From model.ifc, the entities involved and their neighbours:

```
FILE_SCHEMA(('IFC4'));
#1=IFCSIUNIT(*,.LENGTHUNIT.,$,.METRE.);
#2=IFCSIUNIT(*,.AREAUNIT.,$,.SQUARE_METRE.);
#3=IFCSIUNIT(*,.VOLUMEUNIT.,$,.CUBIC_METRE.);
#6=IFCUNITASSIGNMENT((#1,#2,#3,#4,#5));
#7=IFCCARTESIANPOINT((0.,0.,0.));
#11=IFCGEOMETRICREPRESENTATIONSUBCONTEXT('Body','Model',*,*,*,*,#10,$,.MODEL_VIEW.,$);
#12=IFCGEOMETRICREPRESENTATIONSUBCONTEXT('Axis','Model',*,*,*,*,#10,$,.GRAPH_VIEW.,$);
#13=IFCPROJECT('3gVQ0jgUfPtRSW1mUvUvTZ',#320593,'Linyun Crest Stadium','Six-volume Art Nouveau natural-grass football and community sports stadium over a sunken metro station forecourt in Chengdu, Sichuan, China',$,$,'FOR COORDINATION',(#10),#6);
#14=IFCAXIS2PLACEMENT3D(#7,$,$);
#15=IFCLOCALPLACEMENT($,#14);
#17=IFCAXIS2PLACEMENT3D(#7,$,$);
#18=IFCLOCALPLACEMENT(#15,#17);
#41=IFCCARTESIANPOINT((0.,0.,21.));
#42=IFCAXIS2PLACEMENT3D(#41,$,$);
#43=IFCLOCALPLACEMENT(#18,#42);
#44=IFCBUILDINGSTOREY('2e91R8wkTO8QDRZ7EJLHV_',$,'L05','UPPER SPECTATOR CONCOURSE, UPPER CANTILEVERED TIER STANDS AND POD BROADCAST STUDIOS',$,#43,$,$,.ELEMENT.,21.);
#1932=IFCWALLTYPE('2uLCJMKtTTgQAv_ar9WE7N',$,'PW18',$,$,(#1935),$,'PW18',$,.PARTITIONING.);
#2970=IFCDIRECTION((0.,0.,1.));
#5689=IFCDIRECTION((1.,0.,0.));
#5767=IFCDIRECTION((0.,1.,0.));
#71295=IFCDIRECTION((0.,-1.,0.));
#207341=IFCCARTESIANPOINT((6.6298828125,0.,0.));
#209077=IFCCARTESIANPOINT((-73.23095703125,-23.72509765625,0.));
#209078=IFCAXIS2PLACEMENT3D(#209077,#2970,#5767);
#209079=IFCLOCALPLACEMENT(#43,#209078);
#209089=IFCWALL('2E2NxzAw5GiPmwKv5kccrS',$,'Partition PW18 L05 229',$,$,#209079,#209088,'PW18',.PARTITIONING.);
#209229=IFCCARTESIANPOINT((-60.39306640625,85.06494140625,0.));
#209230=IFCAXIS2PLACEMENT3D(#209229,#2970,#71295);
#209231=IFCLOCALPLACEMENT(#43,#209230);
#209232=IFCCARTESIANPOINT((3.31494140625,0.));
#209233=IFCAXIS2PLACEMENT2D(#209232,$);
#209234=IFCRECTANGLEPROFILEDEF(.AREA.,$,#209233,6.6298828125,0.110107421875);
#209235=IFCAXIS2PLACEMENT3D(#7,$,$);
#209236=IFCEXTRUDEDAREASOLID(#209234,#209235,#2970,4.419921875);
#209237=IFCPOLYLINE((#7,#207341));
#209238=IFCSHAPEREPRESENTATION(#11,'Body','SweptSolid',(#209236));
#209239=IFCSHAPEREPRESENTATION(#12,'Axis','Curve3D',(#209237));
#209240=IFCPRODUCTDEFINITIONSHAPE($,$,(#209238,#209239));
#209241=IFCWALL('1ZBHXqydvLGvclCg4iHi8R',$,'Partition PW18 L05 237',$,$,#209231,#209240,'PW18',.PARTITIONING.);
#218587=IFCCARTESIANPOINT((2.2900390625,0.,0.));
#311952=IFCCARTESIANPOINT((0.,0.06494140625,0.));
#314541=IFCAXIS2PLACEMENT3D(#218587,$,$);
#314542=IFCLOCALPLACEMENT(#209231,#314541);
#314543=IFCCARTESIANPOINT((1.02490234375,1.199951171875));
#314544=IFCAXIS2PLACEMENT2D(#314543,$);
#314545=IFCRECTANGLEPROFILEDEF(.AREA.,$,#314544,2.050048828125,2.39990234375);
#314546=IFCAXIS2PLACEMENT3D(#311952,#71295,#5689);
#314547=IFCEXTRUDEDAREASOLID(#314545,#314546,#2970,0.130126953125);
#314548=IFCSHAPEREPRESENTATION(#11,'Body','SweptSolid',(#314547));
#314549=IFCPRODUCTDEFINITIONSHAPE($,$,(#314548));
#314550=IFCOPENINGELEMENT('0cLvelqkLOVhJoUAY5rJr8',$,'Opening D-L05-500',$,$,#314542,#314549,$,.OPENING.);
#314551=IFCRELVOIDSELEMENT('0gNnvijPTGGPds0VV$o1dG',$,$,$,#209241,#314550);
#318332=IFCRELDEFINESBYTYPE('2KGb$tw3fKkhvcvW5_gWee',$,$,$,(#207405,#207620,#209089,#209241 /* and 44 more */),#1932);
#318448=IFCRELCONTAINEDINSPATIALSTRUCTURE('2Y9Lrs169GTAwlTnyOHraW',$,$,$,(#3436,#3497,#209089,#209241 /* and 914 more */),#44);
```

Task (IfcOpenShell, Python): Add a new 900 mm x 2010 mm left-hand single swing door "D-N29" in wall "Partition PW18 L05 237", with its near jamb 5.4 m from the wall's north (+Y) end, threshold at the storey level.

```python
import numpy as np
import ifcopenshell
import ifcopenshell.api.feature
import ifcopenshell.api.geometry
import ifcopenshell.api.root
import ifcopenshell.api.spatial
import ifcopenshell.geom
import ifcopenshell.util.element
import ifcopenshell.util.placement
import ifcopenshell.util.representation
import ifcopenshell.util.shape
import ifcopenshell.util.unit

model = ifcopenshell.open("model.ifc")
unit_scale = ifcopenshell.util.unit.calculate_unit_scale(model)
settings = ifcopenshell.geom.settings()


def volume(element):
    """Net volume in cubic metres, openings subtracted."""
    shape = ifcopenshell.geom.create_shape(settings, element)
    return ifcopenshell.util.shape.get_volume(shape.geometry)


wall = model.by_id(209241)
storey = ifcopenshell.util.element.get_container(wall, ifc_class="IfcBuildingStorey")
context = ifcopenshell.util.representation.get_context(model, "Model", "Body", "MODEL_VIEW")
before = volume(wall)

width, height, from_end, sill = 0.9, 2.01, 5.4, 0.0  # metres

# The wall runs along its own X axis, and the end named is its -X end.
wall_shape = ifcopenshell.geom.create_shape(settings, wall)
x, y, z = ifcopenshell.util.shape.get_vertices(wall_shape.geometry).T
start = x.min() + from_end
face, thickness = float(y.min()), float(y.max() - y.min())
wall_matrix = ifcopenshell.util.placement.get_local_placement(wall.ObjectPlacement)
level = ifcopenshell.util.placement.get_local_placement(storey.ObjectPlacement)[2, 3]


def in_wall(x, y):
    """Placement at x, y metres in the wall's axes, at sill height."""
    matrix = wall_matrix.copy()
    matrix[:, 3] = wall_matrix @ np.array([x / unit_scale, y / unit_scale, 0.0, 1.0])
    matrix[2, 3] = level + sill / unit_scale
    return matrix


# Opening: a box that overshoots both wall faces by 50 mm.
opening = ifcopenshell.api.root.create_entity(model, ifc_class="IfcOpeningElement", predefined_type="OPENING")
box = ifcopenshell.api.geometry.add_wall_representation(
    model, context=context, length=width, height=height, thickness=thickness + 0.1
)
ifcopenshell.api.geometry.assign_representation(model, product=opening, representation=box)
ifcopenshell.api.geometry.edit_object_placement(model, product=opening, matrix=in_wall(start, face - 0.05), is_si=False)
ifcopenshell.api.feature.add_feature(model, feature=opening, element=wall)

door = ifcopenshell.api.root.create_entity(model, ifc_class="IfcDoor", name="D-N29", predefined_type="DOOR")
door.OverallWidth, door.OverallHeight = width / unit_scale, height / unit_scale
door.OperationType = "SINGLE_SWING_LEFT"
body = ifcopenshell.api.geometry.add_door_representation(
    model,
    context=context,
    overall_width=door.OverallWidth,
    overall_height=door.OverallHeight,
    operation_type="SINGLE_SWING_LEFT",
    lining_properties={"LiningDepth": thickness / unit_scale, "ThresholdDepth": thickness / unit_scale},
)
ifcopenshell.api.geometry.assign_representation(model, product=door, representation=body)
ifcopenshell.api.spatial.assign_container(model, products=[door], relating_structure=storey)
ifcopenshell.api.feature.add_filling(model, opening=opening, element=door)

# The lining spans the wall, so the door starts at the wall face.
ifcopenshell.api.geometry.edit_object_placement(model, product=door, matrix=in_wall(start, face), is_si=False)

after = volume(wall)

print(f"wall volume {before:.3f} -> {after:.3f} m3")

model.write("model_updated.ifc")
```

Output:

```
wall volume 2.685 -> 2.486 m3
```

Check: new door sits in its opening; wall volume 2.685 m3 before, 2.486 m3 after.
